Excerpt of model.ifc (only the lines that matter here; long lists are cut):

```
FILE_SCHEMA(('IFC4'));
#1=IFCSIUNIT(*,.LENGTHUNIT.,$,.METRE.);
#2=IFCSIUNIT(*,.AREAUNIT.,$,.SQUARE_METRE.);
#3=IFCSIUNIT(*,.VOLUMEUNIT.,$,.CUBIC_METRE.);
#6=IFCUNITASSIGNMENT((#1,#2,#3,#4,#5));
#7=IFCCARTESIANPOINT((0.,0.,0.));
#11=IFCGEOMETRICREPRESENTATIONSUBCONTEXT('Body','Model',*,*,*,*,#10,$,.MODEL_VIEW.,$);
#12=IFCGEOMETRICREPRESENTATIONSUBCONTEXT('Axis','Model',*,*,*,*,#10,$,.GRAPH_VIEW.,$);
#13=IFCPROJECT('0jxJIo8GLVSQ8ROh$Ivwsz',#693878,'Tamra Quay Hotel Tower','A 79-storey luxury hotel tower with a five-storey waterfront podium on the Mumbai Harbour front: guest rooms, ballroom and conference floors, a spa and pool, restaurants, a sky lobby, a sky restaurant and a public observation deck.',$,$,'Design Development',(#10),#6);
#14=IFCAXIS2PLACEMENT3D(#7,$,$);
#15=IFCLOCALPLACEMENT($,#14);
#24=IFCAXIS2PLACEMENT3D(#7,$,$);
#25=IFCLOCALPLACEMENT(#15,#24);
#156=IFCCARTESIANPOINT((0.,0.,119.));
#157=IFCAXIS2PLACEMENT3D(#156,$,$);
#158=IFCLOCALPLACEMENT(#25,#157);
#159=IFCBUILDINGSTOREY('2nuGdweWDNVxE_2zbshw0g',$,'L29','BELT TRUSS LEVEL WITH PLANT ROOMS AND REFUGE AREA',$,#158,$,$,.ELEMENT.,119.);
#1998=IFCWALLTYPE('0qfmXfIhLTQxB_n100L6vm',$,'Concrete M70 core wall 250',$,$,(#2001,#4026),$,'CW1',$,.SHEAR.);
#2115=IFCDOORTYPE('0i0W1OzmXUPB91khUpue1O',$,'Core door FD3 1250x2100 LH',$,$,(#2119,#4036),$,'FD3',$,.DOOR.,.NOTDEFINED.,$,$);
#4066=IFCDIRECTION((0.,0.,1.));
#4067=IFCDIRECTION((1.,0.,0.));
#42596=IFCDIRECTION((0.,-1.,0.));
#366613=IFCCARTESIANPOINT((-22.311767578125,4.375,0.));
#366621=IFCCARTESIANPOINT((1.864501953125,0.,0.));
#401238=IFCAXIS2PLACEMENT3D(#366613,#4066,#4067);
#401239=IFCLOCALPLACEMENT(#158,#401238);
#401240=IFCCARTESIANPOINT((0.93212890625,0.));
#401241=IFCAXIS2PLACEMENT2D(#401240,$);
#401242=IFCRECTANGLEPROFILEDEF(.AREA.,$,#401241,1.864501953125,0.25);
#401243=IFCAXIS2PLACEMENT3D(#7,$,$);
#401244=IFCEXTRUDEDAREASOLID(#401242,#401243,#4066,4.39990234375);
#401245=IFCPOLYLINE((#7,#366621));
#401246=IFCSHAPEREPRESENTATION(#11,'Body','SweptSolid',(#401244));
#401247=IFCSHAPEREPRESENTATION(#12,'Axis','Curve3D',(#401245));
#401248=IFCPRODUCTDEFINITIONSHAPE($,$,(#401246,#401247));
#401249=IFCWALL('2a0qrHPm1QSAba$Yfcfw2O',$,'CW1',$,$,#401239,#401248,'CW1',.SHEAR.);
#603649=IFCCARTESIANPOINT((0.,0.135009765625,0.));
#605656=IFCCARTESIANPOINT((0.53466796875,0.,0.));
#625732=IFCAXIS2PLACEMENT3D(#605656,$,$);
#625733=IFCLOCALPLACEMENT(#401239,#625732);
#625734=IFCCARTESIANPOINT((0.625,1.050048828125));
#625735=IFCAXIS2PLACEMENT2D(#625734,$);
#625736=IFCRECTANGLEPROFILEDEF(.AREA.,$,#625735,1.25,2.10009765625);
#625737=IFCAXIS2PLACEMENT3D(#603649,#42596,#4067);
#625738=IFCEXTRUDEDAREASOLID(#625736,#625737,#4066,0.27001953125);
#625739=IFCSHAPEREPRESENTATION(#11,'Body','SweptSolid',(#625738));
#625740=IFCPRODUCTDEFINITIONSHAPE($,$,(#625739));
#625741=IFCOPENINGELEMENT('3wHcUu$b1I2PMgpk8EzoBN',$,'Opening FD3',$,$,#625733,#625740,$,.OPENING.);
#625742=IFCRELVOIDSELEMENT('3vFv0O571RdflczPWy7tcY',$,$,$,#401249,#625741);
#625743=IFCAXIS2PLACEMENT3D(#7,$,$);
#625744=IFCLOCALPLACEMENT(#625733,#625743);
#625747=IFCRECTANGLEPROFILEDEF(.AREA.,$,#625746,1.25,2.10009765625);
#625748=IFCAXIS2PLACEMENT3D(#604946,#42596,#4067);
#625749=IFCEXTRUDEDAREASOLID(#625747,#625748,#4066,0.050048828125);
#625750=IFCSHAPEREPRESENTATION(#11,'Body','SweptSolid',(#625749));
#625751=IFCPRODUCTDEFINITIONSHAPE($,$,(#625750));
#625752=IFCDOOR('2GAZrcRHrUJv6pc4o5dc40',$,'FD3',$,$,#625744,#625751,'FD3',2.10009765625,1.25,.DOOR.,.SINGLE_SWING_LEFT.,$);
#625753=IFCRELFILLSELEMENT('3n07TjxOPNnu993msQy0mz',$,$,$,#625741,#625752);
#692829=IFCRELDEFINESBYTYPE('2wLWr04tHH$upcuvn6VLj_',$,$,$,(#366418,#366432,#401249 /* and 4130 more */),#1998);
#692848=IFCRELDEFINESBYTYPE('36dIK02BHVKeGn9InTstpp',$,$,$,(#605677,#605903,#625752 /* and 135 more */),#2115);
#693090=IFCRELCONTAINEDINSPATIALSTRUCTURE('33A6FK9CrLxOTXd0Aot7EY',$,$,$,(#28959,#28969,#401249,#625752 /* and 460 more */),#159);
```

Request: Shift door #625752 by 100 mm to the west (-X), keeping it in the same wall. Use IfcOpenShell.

```python
import ifcopenshell
import ifcopenshell.api.geometry
import ifcopenshell.util.placement
import ifcopenshell.util.unit

model = ifcopenshell.open("model.ifc")
unit_scale = ifcopenshell.util.unit.calculate_unit_scale(model)

door = model.by_guid("2GAZrcRHrUJv6pc4o5dc40")
opening = door.FillsVoids[0].RelatingOpeningElement
wall = opening.VoidsElements[0].RelatingBuildingElement

wall_matrix = ifcopenshell.util.placement.get_local_placement(wall.ObjectPlacement)
shift = wall_matrix[:3, 0] * -0.1 / unit_scale
before = ifcopenshell.util.placement.get_local_placement(door.ObjectPlacement)[:3, 3].copy()

# The door is placed relative to its opening, so it follows when the opening moves.
matrix = ifcopenshell.util.placement.get_local_placement(opening.ObjectPlacement)
matrix[:3, 3] += shift
ifcopenshell.api.geometry.edit_object_placement(
    model, product=opening, matrix=matrix, is_si=False, should_transform_children=True
)

after = ifcopenshell.util.placement.get_local_placement(door.ObjectPlacement)[:3, 3]
print("door moved by", (after - before).round(3) + 0.0)

model.write("model_v2.ifc")
```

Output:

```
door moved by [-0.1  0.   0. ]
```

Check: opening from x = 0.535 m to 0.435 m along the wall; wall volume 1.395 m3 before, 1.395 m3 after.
